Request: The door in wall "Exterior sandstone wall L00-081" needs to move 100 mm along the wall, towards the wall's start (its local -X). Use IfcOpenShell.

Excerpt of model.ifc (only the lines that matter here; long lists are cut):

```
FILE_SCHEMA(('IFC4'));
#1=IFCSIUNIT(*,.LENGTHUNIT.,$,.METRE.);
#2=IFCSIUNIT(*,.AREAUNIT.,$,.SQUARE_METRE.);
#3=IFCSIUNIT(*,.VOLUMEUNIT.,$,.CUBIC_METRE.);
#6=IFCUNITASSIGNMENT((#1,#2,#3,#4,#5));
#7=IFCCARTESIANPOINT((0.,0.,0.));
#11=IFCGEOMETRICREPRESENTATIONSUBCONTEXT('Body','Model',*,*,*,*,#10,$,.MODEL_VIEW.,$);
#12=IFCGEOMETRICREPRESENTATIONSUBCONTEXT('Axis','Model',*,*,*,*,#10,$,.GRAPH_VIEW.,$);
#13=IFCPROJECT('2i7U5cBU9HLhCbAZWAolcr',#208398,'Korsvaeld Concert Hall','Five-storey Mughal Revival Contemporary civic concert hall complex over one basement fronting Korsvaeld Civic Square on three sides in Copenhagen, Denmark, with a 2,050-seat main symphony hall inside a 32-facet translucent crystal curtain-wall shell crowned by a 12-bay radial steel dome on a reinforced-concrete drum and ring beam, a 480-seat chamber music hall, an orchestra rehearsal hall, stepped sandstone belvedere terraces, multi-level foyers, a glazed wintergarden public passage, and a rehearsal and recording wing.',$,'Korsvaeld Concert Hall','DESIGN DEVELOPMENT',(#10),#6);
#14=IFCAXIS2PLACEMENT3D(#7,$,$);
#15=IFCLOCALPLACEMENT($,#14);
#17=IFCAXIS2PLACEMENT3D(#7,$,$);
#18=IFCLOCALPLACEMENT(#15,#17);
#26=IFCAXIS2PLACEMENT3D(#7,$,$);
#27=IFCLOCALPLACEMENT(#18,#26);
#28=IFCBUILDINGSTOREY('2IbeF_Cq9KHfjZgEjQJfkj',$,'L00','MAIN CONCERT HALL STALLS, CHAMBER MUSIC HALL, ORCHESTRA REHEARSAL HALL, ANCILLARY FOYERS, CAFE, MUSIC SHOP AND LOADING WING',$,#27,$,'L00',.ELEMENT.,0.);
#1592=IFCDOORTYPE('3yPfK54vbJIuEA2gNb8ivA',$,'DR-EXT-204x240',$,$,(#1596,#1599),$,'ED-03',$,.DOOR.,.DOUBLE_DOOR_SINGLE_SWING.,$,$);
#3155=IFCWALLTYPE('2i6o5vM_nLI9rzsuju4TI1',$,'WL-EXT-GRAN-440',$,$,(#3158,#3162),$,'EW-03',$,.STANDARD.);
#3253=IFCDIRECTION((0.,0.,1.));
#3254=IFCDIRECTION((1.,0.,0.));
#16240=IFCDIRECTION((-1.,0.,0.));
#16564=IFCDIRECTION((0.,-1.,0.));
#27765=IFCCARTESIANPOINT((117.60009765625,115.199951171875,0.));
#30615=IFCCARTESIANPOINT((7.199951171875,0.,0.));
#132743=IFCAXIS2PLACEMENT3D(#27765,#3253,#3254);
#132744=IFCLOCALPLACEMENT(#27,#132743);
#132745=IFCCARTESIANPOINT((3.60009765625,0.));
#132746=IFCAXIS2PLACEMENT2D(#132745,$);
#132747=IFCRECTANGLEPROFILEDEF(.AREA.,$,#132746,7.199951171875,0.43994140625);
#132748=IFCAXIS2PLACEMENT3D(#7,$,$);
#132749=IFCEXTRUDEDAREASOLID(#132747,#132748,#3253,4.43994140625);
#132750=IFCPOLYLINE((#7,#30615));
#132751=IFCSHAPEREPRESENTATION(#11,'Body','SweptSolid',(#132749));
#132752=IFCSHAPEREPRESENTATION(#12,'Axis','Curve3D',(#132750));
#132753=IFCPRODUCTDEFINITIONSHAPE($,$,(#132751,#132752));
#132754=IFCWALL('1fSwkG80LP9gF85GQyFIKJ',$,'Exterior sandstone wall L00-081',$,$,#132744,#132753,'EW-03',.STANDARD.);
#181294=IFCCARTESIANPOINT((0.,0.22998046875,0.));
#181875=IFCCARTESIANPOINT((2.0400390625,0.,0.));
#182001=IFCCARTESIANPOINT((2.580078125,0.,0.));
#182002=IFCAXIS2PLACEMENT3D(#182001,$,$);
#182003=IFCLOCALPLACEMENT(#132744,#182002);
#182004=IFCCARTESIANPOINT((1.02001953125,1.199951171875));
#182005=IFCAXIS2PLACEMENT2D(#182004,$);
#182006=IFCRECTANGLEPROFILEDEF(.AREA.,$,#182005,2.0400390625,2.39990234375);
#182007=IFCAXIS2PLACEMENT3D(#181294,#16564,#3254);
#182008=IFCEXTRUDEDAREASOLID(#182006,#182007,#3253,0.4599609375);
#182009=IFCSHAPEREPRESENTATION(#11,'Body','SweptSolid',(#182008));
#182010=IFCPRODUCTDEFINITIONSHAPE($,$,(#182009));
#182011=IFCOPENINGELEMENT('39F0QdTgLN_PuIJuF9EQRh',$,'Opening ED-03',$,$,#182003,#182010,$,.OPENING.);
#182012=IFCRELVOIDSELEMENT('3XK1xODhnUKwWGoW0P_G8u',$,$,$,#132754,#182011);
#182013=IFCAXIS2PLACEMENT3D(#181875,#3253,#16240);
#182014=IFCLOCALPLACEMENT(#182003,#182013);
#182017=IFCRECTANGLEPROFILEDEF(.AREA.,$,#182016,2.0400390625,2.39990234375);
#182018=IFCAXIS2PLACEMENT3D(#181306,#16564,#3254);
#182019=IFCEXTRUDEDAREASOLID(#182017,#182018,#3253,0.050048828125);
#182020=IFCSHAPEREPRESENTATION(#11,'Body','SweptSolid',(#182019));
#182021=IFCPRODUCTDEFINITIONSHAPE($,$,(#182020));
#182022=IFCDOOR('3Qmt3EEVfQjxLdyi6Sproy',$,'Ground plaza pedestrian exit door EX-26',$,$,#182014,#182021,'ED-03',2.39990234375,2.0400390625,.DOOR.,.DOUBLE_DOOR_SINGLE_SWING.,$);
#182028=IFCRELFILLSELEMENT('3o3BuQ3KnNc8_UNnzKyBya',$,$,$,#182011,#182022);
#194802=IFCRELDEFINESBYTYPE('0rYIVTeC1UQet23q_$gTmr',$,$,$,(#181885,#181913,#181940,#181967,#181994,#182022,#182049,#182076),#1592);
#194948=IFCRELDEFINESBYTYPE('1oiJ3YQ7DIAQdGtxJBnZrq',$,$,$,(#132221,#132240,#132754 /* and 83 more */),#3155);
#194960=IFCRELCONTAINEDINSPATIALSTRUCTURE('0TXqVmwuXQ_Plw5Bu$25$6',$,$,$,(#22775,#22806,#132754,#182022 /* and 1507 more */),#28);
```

```python
import ifcopenshell
import ifcopenshell.api.geometry
import ifcopenshell.util.placement
import ifcopenshell.util.unit

model = ifcopenshell.open("model.ifc")
unit_scale = ifcopenshell.util.unit.calculate_unit_scale(model)

door = model.by_id(182022)
opening = door.FillsVoids[0].RelatingOpeningElement
wall = opening.VoidsElements[0].RelatingBuildingElement

wall_matrix = ifcopenshell.util.placement.get_local_placement(wall.ObjectPlacement)
shift = wall_matrix[:3, 0] * -0.1 / unit_scale
before = ifcopenshell.util.placement.get_local_placement(door.ObjectPlacement)[:3, 3].copy()

# The door is placed relative to its opening, so it follows when the opening moves.
matrix = ifcopenshell.util.placement.get_local_placement(opening.ObjectPlacement)
matrix[:3, 3] += shift
ifcopenshell.api.geometry.edit_object_placement(
    model, product=opening, matrix=matrix, is_si=False, should_transform_children=True
)

after = ifcopenshell.util.placement.get_local_placement(door.ObjectPlacement)[:3, 3]
print("door moved by", (after - before).round(3) + 0.0)

model.write("model_updated.ifc")
```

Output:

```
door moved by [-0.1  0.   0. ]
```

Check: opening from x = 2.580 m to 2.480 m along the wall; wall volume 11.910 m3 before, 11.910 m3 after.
